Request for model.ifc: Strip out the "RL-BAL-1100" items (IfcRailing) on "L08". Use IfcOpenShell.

First a look at what the model holds.

```python
import ifcopenshell
import ifcopenshell.util.element

model = ifcopenshell.open("model.ifc")
print(model.schema)
storey = next(s for s in model.by_type("IfcBuildingStorey") if s.Name == "L08")
railings = [e for e in ifcopenshell.util.element.get_decomposition(storey) if e.is_a("IfcRailing")]
seen = {}
for e in railings:
    element_type = ifcopenshell.util.element.get_type(e)
    name = element_type.Name if element_type not in (None, e) else None
    seen[name] = seen.get(name, 0) + 1
for name, count in sorted(seen.items(), key=str):
    print(count, "x", name)
```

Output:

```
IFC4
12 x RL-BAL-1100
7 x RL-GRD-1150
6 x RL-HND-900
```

```python
import ifcopenshell
import ifcopenshell.api.root
import ifcopenshell.util.element

model = ifcopenshell.open("model.ifc")

storey = next(s for s in model.by_type("IfcBuildingStorey") if s.Name == "L08")
railings = [e for e in ifcopenshell.util.element.get_decomposition(storey) if e.is_a("IfcRailing")]
targets = [e for e in railings if (t := ifcopenshell.util.element.get_type(e)) not in (None, e) and t.Name == "RL-BAL-1100"]

for e in targets:
    ifcopenshell.api.root.remove_product(model, product=e)
print(len(targets), "removed")

model.write("model_edited.ifc")
```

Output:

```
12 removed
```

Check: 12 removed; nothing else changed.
